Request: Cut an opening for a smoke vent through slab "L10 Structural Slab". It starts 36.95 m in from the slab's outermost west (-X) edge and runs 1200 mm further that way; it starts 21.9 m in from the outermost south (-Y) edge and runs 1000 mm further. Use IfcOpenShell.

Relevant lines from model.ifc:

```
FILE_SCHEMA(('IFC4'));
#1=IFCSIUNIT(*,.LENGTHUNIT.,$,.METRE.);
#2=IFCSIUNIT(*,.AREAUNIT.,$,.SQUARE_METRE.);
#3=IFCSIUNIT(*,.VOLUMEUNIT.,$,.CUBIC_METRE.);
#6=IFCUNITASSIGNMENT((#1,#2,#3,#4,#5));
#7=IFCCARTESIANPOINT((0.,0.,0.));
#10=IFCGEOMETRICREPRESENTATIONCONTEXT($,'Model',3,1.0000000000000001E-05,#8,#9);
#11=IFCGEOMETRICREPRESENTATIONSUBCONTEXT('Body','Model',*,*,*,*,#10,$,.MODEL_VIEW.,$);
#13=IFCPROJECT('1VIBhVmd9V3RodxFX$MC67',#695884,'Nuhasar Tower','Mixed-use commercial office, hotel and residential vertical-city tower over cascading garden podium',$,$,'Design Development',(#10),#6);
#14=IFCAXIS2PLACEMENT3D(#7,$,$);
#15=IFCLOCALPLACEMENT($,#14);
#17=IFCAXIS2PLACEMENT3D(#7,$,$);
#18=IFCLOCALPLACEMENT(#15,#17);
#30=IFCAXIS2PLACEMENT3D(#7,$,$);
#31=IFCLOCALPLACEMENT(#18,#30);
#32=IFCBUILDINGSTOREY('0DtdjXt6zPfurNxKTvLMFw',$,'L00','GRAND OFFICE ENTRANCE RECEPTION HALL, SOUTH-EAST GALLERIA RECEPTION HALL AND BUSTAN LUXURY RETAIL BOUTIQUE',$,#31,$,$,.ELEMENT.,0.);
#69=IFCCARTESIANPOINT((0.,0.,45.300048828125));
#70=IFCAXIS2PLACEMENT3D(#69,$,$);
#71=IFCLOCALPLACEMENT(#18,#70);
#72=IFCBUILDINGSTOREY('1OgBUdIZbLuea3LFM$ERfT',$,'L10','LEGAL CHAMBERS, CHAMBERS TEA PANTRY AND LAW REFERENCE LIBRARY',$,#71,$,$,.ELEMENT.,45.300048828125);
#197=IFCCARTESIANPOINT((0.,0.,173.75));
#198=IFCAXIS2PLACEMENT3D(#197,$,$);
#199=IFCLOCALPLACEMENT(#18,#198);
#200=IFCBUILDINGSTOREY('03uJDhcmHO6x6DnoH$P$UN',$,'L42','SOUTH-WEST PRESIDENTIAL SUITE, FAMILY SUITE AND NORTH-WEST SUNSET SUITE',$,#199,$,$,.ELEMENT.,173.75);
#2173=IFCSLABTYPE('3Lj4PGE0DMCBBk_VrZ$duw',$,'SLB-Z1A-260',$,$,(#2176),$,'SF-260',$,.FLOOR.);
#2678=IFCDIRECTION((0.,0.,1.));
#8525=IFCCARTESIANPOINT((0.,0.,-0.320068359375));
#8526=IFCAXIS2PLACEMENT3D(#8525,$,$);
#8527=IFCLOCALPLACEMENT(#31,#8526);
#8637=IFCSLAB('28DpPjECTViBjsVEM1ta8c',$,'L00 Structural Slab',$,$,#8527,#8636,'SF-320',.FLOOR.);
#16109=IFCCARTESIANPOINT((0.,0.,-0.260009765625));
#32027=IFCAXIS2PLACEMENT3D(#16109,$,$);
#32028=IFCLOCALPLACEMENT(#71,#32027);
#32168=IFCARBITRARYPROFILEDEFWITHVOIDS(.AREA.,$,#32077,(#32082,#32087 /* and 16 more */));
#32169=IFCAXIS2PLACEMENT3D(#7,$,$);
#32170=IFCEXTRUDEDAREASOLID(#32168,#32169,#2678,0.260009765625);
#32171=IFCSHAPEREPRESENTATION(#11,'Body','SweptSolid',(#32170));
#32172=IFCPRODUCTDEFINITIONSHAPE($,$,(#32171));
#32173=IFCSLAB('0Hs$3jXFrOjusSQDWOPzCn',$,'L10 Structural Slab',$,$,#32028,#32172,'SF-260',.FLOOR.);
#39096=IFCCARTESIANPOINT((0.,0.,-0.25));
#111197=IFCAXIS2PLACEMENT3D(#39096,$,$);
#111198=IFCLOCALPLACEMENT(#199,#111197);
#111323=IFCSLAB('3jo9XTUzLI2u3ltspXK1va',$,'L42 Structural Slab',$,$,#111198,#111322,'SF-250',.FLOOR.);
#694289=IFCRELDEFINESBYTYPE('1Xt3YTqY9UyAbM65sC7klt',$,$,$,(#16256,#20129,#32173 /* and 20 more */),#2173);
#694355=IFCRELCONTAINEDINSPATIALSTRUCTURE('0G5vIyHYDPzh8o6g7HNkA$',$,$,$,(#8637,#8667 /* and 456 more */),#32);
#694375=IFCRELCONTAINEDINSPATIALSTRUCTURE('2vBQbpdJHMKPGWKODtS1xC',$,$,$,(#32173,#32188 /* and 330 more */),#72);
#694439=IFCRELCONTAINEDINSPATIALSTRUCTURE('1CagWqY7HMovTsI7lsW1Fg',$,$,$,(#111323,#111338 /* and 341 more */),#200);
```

```python
import numpy as np
import ifcopenshell
import ifcopenshell.api.feature
import ifcopenshell.api.geometry
import ifcopenshell.api.root
import ifcopenshell.geom
import ifcopenshell.util.placement
import ifcopenshell.util.representation
import ifcopenshell.util.shape
import ifcopenshell.util.unit

model = ifcopenshell.open("model.ifc")
unit_scale = ifcopenshell.util.unit.calculate_unit_scale(model)
settings = ifcopenshell.geom.settings()


def volume(element):
    """Net volume in cubic metres, openings subtracted."""
    shape = ifcopenshell.geom.create_shape(settings, element)
    return ifcopenshell.util.shape.get_volume(shape.geometry)


slab = model.by_id(32173)
before = volume(slab)

# Extent in the slab's own axes, in metres. The edges named are its -X and -Y sides.
slab_shape = ifcopenshell.geom.create_shape(settings, slab)
vertices = ifcopenshell.util.shape.get_vertices(slab_shape.geometry)
x_min, y_min, bottom = vertices.min(axis=0)
top = vertices[:, 2].max()

opening = ifcopenshell.api.root.create_entity(model, ifc_class="IfcOpeningElement", name="Smoke vent opening", predefined_type="OPENING")
context = ifcopenshell.util.representation.get_context(model, "Model", "Body", "MODEL_VIEW")
width, depth = 1.2, 1
outline = [(0.0, 0.0), (width, 0.0), (width, depth), (0.0, depth), (0.0, 0.0)]
# Overshoot both faces by 50 mm so the cut is clean.
shape = ifcopenshell.api.geometry.add_slab_representation(
    model, context=context, depth=top - bottom + 0.1, polyline=outline
)
ifcopenshell.api.geometry.assign_representation(model, product=opening, representation=shape)

matrix = ifcopenshell.util.placement.get_local_placement(slab.ObjectPlacement)
matrix[:, 3] = matrix @ np.append(np.array([x_min + 36.95, y_min + 21.9, bottom - 0.05]) / unit_scale, 1.0)
ifcopenshell.api.geometry.edit_object_placement(model, product=opening, matrix=matrix, is_si=False)
ifcopenshell.api.feature.add_feature(model, feature=opening, element=slab)

after = volume(slab)

print(f"slab volume {before:.3f} -> {after:.3f} m3")

model.write("model_rev.ifc")
```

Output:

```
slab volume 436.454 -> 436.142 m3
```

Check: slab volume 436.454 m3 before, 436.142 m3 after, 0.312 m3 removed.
